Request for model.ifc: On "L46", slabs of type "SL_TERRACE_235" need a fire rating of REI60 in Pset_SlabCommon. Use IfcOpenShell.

First a look at what the model holds.

```python
import ifcopenshell
import ifcopenshell.util.element

model = ifcopenshell.open("model.ifc")
print(model.schema)
storey = next(s for s in model.by_type("IfcBuildingStorey") if s.Name == "L46")
slabs = [e for e in ifcopenshell.util.element.get_decomposition(storey) if e.is_a("IfcSlab")]
seen = {}
for e in slabs:
    element_type = ifcopenshell.util.element.get_type(e)
    key = (element_type.Name if element_type != e and element_type else None, ifcopenshell.util.element.get_pset(e, "Pset_SlabCommon", "FireRating"))
    seen[key] = seen.get(key, 0) + 1
for (name, value), count in sorted(seen.items(), key=str):
    print(count, "x", name, "|", value)
```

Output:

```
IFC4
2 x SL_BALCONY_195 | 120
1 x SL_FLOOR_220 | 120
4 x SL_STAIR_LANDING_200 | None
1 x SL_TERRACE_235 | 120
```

```python
import ifcopenshell
import ifcopenshell.api.pset
import ifcopenshell.util.element

model = ifcopenshell.open("model.ifc")

storey = next(s for s in model.by_type("IfcBuildingStorey") if s.Name == "L46")
slabs = [e for e in ifcopenshell.util.element.get_decomposition(storey) if e.is_a("IfcSlab")]

count = 0
for e in slabs:
    element_type = ifcopenshell.util.element.get_type(e)
    if element_type in (None, e) or element_type.Name != "SL_TERRACE_235":
        continue
    found = ifcopenshell.util.element.get_pset(e, "Pset_SlabCommon", should_inherit=False)
    if found:
        pset = model.by_id(found["id"])
        if len(ifcopenshell.util.element.get_elements_by_pset(pset)) > 1:
            pset = ifcopenshell.api.pset.unshare_pset(model, products=[e], pset=pset)[0]
    else:
        pset = ifcopenshell.api.pset.add_pset(model, product=e, name="Pset_SlabCommon")
    ifcopenshell.api.pset.edit_pset(model, pset=pset, properties={"FireRating": "REI60"})
    count += 1

print(count, "slabs updated")

model.write("model-out.ifc")
```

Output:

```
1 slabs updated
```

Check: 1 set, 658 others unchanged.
